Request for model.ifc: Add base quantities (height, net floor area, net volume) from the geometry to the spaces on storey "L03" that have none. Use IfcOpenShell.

First a look at what the model holds.

```python
import ifcopenshell
import ifcopenshell.util.element
import ifcopenshell.util.unit

model = ifcopenshell.open("model.ifc")
print(model.schema)
for unit_type in ("LENGTHUNIT", "AREAUNIT", "VOLUMEUNIT"):
    print(unit_type, ifcopenshell.util.unit.calculate_unit_scale(model, unit_type))
storey = next(s for s in model.by_type("IfcBuildingStorey") if s.Name == "L03")
spaces = [e for e in ifcopenshell.util.element.get_decomposition(storey) if e.is_a("IfcSpace")]
for e in sorted(spaces, key=lambda e: e.id()):
    print(e.id(), e.is_a(), e.Name, list(ifcopenshell.util.element.get_psets(e, qtos_only=True)), sep=" | ")
```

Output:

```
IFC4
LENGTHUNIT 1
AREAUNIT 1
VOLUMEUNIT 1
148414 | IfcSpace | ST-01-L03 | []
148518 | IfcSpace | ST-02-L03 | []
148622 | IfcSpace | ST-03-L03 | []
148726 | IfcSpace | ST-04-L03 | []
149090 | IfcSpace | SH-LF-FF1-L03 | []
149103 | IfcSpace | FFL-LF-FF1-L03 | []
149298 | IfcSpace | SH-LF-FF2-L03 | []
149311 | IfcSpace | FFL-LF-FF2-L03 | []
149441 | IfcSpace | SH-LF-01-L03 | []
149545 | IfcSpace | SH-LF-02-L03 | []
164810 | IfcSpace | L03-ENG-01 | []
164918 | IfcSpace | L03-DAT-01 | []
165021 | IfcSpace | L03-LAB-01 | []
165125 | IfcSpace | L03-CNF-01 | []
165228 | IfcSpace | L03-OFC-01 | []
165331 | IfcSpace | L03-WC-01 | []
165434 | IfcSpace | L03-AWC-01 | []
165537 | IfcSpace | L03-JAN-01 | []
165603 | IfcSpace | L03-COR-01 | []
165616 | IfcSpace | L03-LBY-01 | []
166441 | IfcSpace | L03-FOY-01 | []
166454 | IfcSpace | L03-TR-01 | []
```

```python
import ifcopenshell
import ifcopenshell.api.pset
import ifcopenshell.geom
import ifcopenshell.util.element
import ifcopenshell.util.shape
import ifcopenshell.util.unit

model = ifcopenshell.open("model.ifc")
unit_scale = ifcopenshell.util.unit.calculate_unit_scale(model)
area_scale = ifcopenshell.util.unit.calculate_unit_scale(model, "AREAUNIT")
volume_scale = ifcopenshell.util.unit.calculate_unit_scale(model, "VOLUMEUNIT")
settings = ifcopenshell.geom.settings()

storey = next(s for s in model.by_type("IfcBuildingStorey") if s.Name == "L03")
spaces = [e for e in ifcopenshell.util.element.get_decomposition(storey) if e.is_a("IfcSpace")]

for e in sorted(spaces, key=lambda e: e.id()):
    if ifcopenshell.util.element.get_psets(e, qtos_only=True, should_inherit=False):
        continue
    # Geometry comes back in metres, in the element's own axes.
    shape = ifcopenshell.geom.create_shape(settings, e)
    values = {
        "Height": ifcopenshell.util.shape.get_z(shape.geometry) / unit_scale,
        "NetFloorArea": ifcopenshell.util.shape.get_footprint_area(shape.geometry) / area_scale,
        "NetVolume": ifcopenshell.util.shape.get_volume(shape.geometry) / volume_scale,
    }
    qto = ifcopenshell.api.pset.add_qto(model, product=e, name="Qto_SpaceBaseQuantities")
    ifcopenshell.api.pset.edit_qto(model, qto=qto, properties=values)
    print(e.id(), {k: round(v, 3) for k, v in values.items()})

model.write("model_rev.ifc")
```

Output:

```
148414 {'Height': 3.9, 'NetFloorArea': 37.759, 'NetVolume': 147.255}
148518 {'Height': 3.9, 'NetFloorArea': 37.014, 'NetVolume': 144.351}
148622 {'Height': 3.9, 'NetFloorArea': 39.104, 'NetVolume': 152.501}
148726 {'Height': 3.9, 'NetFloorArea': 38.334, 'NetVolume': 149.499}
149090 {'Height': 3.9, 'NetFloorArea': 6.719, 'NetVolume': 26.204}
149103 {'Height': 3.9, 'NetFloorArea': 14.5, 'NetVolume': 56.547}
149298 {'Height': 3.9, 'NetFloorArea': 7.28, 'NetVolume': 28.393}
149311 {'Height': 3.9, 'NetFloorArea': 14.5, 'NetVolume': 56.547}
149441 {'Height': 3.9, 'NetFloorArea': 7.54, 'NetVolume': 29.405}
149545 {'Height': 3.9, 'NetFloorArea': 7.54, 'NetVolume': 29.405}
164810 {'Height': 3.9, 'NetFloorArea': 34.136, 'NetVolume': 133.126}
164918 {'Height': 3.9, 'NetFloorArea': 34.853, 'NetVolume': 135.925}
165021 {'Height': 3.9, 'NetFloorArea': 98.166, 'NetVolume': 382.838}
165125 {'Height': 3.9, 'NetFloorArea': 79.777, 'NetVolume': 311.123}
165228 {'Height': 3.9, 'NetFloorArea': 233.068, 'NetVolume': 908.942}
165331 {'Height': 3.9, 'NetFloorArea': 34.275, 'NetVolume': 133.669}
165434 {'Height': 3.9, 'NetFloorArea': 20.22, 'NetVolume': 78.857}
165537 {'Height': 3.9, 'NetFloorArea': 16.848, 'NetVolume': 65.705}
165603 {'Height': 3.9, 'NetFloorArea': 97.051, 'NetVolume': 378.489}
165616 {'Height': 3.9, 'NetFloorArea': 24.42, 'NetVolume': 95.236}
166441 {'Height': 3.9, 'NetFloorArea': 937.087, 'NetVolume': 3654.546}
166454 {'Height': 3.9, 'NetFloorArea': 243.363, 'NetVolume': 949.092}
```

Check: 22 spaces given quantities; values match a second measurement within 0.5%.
